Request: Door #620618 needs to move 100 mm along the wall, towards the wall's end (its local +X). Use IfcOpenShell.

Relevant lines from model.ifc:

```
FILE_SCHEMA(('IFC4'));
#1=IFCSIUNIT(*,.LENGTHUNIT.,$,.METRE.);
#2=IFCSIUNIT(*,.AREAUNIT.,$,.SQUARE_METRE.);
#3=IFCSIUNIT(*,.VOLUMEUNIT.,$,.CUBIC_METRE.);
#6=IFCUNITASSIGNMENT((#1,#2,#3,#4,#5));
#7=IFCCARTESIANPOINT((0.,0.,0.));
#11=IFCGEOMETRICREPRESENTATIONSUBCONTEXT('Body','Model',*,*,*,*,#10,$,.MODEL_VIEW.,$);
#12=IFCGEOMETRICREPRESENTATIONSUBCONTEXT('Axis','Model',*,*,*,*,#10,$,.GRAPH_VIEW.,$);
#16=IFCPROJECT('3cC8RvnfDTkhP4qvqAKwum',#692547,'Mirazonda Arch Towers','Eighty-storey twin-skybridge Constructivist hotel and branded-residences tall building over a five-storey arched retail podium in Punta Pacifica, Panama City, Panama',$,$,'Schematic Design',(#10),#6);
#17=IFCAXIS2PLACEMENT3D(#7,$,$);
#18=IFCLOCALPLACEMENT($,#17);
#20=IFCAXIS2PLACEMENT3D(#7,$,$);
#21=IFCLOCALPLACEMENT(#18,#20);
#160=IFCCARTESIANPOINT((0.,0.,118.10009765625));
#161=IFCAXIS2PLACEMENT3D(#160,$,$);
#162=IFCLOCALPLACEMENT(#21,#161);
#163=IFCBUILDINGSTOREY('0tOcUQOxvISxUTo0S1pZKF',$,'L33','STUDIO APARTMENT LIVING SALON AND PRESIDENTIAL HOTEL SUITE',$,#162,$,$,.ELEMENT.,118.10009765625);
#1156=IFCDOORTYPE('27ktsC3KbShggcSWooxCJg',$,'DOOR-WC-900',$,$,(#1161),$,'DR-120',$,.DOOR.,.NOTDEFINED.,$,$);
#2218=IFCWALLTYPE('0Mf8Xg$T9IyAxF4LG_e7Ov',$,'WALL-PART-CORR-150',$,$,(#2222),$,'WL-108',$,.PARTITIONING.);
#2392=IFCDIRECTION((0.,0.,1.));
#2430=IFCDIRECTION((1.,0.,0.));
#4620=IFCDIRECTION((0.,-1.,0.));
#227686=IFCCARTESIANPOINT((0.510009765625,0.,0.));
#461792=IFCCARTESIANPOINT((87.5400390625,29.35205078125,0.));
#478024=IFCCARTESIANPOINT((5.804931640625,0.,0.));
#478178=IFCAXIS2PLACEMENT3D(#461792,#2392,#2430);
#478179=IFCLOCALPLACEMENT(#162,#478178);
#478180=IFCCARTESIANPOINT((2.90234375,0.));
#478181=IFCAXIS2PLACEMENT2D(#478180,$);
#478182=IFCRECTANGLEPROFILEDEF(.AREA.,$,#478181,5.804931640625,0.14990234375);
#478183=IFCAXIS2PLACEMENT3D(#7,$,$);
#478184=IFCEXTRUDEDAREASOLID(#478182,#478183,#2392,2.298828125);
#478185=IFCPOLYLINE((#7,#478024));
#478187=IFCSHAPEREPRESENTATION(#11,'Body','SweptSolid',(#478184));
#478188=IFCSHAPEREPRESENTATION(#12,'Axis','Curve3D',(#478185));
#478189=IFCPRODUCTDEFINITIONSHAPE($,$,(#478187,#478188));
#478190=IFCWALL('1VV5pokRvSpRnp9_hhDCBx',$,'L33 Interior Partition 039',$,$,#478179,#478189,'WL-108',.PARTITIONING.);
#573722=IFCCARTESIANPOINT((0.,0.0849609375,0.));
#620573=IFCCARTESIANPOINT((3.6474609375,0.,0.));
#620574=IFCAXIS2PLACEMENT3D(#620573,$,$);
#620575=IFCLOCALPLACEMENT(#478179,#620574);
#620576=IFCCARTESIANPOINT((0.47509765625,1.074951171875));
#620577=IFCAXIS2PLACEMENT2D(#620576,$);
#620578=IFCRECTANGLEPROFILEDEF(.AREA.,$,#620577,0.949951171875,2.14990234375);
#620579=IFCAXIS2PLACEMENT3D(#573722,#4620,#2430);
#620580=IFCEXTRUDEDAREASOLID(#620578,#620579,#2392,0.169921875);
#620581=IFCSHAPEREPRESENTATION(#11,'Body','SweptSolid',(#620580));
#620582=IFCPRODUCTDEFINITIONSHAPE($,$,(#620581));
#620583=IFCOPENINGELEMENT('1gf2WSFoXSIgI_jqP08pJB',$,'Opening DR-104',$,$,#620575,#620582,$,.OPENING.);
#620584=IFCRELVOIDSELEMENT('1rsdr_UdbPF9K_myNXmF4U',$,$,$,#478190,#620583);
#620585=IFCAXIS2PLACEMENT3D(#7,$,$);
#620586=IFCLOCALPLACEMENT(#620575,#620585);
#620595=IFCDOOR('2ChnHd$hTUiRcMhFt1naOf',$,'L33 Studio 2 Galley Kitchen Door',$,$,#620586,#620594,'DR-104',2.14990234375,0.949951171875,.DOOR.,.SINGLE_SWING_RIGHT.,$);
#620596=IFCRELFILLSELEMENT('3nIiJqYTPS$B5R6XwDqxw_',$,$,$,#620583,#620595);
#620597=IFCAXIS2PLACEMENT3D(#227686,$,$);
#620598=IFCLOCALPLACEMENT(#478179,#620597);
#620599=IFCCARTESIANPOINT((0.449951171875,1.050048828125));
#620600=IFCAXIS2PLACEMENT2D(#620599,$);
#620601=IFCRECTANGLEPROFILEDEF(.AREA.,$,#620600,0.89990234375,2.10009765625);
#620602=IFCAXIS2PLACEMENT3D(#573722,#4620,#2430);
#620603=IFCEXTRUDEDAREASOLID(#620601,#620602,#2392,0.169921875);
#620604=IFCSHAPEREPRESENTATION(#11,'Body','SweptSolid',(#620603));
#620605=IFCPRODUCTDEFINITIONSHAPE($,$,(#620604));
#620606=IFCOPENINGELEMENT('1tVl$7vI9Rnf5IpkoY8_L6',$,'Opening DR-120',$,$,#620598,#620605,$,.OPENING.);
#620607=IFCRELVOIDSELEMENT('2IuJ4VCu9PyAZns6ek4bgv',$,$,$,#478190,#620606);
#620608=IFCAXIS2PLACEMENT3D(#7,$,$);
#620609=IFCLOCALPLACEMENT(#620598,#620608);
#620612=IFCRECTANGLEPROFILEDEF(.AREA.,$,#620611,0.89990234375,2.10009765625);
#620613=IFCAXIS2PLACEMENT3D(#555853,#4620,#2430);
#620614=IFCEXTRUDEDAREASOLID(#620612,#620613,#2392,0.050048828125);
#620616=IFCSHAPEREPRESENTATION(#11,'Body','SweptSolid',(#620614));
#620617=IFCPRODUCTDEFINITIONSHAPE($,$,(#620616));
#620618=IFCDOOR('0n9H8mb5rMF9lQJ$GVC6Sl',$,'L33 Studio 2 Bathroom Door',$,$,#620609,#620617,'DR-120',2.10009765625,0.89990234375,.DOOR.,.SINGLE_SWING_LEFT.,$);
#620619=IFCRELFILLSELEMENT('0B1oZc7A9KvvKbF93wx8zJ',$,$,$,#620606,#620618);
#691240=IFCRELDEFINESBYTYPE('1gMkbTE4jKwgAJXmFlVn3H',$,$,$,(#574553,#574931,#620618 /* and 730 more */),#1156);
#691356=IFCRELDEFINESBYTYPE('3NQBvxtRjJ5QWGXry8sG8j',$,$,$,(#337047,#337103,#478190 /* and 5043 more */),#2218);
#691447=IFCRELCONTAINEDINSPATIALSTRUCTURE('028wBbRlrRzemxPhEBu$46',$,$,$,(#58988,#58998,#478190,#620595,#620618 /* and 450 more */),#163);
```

```python
import ifcopenshell
import ifcopenshell.api.geometry
import ifcopenshell.util.placement

model = ifcopenshell.open("model.ifc")

door = model.by_id(620618)
opening = door.FillsVoids[0].RelatingOpeningElement
wall = opening.VoidsElements[0].RelatingBuildingElement

wall_matrix = ifcopenshell.util.placement.get_local_placement(wall.ObjectPlacement)
shift = wall_matrix[:3, 0] * 0.1
before = ifcopenshell.util.placement.get_local_placement(door.ObjectPlacement)[:3, 3].copy()

# The door is placed relative to its opening, so it follows when the opening moves.
matrix = ifcopenshell.util.placement.get_local_placement(opening.ObjectPlacement)
matrix[:3, 3] += shift
ifcopenshell.api.geometry.edit_object_placement(
    model, product=opening, matrix=matrix, is_si=False, should_transform_children=True
)

after = ifcopenshell.util.placement.get_local_placement(door.ObjectPlacement)[:3, 3]
print("door moved by", (after - before).round(3) + 0.0)

model.write("model_rev.ifc")
```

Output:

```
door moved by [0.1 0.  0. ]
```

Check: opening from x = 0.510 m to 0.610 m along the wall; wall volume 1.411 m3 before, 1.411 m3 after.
